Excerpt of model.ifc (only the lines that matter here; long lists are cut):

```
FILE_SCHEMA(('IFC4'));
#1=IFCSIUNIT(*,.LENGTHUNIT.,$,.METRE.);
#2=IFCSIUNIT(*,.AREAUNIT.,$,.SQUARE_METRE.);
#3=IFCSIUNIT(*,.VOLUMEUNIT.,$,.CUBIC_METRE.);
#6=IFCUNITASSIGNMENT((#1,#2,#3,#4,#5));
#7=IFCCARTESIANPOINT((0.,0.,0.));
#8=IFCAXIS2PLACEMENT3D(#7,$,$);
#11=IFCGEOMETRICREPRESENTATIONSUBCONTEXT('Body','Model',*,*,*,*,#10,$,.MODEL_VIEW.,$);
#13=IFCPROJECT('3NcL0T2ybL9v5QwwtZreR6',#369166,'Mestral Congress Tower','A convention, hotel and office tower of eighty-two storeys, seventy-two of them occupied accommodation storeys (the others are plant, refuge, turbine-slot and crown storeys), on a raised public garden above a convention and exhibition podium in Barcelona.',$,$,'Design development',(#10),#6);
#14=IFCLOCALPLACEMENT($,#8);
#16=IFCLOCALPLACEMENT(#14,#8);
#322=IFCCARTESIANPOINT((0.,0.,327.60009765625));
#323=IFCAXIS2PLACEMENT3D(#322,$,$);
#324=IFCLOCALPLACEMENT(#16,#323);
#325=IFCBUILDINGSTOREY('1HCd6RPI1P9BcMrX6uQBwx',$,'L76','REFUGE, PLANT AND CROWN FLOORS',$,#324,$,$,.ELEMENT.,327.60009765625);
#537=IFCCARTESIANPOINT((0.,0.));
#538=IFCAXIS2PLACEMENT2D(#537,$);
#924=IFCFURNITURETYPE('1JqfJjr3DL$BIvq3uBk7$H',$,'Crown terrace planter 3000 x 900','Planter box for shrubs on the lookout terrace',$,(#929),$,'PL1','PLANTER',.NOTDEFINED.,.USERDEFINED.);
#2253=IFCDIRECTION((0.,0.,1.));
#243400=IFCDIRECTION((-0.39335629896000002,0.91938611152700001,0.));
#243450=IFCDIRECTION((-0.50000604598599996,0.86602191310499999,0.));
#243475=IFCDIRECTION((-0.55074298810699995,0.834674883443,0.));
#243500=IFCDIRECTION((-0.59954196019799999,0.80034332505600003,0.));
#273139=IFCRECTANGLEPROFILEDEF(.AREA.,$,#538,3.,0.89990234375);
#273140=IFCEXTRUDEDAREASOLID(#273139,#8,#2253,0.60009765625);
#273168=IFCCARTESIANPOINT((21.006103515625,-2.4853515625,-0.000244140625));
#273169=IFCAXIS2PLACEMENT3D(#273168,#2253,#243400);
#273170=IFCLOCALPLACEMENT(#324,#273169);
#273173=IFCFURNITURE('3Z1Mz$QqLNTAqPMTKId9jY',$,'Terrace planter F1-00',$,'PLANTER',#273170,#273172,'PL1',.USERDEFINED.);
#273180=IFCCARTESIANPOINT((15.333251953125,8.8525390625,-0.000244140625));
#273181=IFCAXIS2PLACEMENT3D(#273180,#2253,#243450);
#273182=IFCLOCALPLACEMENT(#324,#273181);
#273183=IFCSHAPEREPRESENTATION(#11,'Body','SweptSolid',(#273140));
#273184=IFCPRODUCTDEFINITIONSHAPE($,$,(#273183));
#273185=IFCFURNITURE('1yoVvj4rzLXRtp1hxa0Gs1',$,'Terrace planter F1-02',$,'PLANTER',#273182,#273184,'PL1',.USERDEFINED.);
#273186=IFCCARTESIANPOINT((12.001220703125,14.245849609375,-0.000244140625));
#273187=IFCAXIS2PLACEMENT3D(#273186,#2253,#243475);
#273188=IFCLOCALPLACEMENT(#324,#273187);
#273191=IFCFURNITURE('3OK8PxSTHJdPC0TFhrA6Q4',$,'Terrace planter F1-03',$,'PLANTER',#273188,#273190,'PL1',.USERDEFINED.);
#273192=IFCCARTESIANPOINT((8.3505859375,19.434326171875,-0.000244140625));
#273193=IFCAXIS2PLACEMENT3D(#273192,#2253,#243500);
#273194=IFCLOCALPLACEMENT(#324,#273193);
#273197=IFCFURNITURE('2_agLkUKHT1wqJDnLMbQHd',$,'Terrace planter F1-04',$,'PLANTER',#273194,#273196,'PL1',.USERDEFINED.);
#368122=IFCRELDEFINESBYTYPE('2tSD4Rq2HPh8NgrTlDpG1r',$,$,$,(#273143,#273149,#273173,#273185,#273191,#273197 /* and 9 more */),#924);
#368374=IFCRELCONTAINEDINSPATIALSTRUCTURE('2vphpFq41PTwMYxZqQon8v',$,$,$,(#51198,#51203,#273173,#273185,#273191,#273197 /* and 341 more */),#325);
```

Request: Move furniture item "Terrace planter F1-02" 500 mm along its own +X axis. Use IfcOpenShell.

```python
import ifcopenshell
import ifcopenshell.api.geometry
import ifcopenshell.util.placement

model = ifcopenshell.open("model.ifc")

item = model.by_guid("1yoVvj4rzLXRtp1hxa0Gs1")
matrix = ifcopenshell.util.placement.get_local_placement(item.ObjectPlacement)
matrix[:3, 3] += matrix[:3, 0] * 0.5
ifcopenshell.api.geometry.edit_object_placement(model, product=item, matrix=matrix, is_si=False)

print(ifcopenshell.util.placement.get_local_placement(item.ObjectPlacement).round(3) + 0.0)

model.write("model_updated.ifc")
```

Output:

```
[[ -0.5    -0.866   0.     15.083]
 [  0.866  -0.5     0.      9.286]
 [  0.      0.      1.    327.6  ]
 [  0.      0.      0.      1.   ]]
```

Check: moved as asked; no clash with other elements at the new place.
